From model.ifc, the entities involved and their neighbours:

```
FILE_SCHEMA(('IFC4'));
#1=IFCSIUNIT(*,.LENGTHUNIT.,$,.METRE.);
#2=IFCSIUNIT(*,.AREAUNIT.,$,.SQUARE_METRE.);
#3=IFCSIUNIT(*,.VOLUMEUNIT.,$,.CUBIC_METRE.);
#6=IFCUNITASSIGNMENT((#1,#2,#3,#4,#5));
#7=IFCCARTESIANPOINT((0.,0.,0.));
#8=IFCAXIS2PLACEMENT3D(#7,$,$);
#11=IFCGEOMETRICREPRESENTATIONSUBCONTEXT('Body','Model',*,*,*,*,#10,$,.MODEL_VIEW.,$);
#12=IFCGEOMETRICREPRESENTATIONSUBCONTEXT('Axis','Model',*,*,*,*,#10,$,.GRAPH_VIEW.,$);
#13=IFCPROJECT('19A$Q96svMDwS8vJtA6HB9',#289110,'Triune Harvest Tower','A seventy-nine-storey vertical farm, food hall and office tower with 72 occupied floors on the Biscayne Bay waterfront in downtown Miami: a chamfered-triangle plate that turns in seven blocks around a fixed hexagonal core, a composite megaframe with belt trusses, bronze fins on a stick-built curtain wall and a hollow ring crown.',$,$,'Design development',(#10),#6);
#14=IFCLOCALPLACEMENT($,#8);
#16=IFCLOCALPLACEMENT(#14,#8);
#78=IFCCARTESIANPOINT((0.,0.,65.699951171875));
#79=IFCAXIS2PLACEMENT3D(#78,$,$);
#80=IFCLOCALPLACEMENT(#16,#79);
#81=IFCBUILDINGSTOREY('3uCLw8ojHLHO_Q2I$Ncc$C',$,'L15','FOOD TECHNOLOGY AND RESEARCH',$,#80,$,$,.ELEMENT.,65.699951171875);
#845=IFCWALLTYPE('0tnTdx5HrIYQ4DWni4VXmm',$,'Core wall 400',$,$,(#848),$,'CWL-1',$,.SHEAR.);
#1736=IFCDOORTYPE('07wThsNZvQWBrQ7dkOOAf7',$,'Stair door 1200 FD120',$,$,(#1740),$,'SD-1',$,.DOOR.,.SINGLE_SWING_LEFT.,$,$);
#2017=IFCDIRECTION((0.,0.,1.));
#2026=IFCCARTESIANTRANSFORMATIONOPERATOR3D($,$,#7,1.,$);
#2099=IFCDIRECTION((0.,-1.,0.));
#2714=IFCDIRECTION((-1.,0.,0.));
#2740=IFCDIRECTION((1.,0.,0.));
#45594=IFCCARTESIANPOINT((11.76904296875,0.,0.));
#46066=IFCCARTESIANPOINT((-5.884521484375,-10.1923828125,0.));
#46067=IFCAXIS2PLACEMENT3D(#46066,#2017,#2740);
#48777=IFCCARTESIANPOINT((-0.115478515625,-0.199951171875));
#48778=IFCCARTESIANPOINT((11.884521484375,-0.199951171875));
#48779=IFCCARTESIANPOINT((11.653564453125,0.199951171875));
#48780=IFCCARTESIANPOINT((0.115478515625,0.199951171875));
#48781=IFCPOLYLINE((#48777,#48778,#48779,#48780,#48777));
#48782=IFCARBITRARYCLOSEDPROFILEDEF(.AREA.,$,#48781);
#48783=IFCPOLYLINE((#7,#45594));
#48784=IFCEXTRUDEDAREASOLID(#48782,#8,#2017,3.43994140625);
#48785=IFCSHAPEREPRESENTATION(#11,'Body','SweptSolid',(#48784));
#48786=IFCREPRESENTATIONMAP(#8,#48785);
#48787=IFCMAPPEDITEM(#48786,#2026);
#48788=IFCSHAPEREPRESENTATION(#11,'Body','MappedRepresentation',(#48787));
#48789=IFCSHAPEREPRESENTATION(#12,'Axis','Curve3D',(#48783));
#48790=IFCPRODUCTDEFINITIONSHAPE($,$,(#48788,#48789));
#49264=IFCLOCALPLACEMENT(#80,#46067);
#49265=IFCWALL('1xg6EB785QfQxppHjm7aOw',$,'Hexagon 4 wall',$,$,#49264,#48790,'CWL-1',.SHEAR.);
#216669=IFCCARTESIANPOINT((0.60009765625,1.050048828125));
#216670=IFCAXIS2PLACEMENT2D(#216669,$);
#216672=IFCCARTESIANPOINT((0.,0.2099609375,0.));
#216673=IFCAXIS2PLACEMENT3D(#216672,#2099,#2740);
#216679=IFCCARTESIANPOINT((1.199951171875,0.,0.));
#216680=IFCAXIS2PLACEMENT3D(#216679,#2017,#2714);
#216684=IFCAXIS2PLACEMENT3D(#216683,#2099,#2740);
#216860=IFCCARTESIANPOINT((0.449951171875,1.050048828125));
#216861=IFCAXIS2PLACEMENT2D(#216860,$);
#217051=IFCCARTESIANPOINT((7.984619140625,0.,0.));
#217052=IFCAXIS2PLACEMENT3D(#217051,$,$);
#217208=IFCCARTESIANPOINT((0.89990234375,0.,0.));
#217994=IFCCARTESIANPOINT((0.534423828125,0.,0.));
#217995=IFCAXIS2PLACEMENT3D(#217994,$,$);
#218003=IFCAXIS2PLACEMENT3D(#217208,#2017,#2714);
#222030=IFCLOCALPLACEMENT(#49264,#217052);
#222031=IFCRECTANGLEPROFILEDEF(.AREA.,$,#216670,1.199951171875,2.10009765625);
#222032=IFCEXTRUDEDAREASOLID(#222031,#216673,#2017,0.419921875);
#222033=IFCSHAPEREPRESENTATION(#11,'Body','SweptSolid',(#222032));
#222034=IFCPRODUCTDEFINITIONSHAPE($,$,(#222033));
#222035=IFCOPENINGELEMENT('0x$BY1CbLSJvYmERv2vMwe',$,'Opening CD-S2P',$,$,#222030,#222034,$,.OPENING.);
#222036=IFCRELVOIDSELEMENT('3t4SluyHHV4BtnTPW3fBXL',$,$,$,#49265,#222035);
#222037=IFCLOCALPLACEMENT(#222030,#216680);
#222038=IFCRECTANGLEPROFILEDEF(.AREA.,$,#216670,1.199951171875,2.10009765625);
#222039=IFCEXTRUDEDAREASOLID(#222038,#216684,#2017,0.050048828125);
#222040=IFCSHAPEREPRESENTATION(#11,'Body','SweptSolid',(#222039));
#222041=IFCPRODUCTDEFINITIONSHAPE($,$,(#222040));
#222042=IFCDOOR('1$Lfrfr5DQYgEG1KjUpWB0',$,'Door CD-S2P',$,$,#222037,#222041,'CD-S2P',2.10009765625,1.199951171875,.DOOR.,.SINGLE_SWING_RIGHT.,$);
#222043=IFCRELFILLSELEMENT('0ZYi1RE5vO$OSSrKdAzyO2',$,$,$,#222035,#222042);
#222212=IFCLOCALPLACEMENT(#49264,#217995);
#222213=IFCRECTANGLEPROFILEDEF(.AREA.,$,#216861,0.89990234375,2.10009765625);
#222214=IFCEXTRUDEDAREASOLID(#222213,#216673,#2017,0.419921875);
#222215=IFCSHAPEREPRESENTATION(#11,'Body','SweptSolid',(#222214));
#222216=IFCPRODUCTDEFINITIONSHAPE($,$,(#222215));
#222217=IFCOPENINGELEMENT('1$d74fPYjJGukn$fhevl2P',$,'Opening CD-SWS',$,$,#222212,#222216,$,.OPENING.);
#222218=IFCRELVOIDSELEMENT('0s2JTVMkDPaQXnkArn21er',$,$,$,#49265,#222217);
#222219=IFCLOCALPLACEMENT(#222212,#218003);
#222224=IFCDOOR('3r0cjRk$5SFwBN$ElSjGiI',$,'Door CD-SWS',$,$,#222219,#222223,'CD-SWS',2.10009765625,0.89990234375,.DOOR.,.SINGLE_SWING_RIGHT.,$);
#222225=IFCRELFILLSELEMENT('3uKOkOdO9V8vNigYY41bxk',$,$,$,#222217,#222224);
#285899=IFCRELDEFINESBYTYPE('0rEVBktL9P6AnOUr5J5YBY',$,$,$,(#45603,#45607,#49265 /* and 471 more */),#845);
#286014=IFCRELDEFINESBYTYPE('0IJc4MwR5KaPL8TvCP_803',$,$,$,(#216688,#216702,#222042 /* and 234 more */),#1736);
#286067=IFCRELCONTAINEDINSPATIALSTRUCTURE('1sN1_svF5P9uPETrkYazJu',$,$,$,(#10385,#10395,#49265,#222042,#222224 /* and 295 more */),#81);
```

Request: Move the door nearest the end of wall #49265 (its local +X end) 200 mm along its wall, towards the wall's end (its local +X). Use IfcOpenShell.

```python
import ifcopenshell
import ifcopenshell.api.geometry
import ifcopenshell.util.placement
import ifcopenshell.util.unit

model = ifcopenshell.open("model.ifc")
unit_scale = ifcopenshell.util.unit.calculate_unit_scale(model)

door = model.by_guid("1$Lfrfr5DQYgEG1KjUpWB0")
opening = door.FillsVoids[0].RelatingOpeningElement
wall = opening.VoidsElements[0].RelatingBuildingElement

wall_matrix = ifcopenshell.util.placement.get_local_placement(wall.ObjectPlacement)
shift = wall_matrix[:3, 0] * 0.2 / unit_scale
before = ifcopenshell.util.placement.get_local_placement(door.ObjectPlacement)[:3, 3].copy()

# The door is placed relative to its opening, so it follows when the opening moves.
matrix = ifcopenshell.util.placement.get_local_placement(opening.ObjectPlacement)
matrix[:3, 3] += shift
ifcopenshell.api.geometry.edit_object_placement(
    model, product=opening, matrix=matrix, is_si=False, should_transform_children=True
)

after = ifcopenshell.util.placement.get_local_placement(door.ObjectPlacement)[:3, 3]
print("door moved by", (after - before).round(3) + 0.0)

model.write("model_v2.ifc")
```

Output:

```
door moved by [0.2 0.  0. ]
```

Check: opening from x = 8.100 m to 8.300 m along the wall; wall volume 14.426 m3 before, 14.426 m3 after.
